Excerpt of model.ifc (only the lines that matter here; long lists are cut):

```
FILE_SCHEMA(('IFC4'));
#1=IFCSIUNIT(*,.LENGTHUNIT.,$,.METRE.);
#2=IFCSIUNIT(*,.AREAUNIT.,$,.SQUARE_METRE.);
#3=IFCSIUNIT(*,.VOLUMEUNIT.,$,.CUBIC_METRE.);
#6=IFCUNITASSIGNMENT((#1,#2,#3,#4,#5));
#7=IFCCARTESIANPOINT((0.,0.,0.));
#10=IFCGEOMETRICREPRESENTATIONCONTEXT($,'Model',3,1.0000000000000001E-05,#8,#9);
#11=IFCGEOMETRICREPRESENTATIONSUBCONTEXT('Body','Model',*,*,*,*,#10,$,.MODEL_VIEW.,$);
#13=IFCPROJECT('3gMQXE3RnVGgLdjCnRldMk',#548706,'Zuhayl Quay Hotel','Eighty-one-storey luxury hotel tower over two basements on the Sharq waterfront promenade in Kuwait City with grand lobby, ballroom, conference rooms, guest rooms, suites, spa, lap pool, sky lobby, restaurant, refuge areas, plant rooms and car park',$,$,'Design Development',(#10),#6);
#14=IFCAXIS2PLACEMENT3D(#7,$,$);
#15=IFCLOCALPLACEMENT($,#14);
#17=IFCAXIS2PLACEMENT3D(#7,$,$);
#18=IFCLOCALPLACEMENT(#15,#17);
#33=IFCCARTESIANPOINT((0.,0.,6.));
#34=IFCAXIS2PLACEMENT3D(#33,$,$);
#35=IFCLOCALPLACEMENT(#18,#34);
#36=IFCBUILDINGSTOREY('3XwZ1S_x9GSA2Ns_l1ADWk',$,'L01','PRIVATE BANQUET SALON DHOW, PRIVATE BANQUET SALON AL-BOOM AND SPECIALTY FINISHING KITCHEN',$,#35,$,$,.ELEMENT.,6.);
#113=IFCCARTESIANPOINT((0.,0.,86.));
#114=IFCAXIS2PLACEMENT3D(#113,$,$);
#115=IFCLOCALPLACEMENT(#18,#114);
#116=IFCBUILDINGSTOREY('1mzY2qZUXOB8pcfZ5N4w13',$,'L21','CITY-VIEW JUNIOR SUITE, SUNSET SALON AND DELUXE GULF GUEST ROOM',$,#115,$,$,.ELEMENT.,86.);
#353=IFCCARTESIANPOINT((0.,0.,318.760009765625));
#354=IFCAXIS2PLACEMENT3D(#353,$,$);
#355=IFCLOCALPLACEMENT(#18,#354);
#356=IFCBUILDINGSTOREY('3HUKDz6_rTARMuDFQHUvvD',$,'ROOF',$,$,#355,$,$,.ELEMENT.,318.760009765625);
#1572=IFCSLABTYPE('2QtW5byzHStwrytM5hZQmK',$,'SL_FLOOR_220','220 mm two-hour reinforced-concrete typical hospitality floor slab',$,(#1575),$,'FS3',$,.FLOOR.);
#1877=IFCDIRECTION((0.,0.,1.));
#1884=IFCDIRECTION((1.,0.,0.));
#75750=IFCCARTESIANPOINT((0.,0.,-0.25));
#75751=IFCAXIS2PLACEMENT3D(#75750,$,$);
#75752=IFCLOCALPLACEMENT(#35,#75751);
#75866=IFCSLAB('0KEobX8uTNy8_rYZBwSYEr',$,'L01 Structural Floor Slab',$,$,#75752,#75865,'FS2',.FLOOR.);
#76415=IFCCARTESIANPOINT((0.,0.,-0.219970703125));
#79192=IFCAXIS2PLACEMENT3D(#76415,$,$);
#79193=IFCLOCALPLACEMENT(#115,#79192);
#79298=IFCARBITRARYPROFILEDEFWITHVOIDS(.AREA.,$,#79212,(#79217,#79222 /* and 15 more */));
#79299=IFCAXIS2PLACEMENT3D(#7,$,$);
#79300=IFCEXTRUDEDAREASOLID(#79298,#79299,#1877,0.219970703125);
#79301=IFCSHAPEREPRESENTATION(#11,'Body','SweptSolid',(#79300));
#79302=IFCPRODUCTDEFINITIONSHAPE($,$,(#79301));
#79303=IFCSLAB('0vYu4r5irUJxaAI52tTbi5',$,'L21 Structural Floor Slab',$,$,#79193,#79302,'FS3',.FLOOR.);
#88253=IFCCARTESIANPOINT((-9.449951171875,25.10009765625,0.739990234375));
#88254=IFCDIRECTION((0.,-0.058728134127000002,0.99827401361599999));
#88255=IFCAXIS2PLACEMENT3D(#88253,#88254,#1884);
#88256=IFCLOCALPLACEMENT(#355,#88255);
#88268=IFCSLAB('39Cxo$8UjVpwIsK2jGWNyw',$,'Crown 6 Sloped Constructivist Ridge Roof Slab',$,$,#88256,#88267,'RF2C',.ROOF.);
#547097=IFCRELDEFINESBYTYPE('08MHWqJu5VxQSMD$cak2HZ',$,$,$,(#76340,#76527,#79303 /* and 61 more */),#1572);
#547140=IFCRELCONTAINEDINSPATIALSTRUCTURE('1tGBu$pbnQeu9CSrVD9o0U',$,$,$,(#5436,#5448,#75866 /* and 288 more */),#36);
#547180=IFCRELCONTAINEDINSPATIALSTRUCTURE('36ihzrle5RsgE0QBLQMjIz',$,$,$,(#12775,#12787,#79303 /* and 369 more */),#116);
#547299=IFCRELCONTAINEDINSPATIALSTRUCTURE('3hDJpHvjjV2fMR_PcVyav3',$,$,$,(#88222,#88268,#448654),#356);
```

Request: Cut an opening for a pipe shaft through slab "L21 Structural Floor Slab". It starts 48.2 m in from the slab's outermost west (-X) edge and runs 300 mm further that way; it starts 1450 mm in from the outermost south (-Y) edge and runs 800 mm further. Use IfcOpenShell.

```python
import numpy as np
import ifcopenshell
import ifcopenshell.api.feature
import ifcopenshell.api.geometry
import ifcopenshell.api.root
import ifcopenshell.geom
import ifcopenshell.util.placement
import ifcopenshell.util.representation
import ifcopenshell.util.shape
import ifcopenshell.util.unit

model = ifcopenshell.open("model.ifc")
unit_scale = ifcopenshell.util.unit.calculate_unit_scale(model)
settings = ifcopenshell.geom.settings()


def volume(element):
    """Net volume in cubic metres, openings subtracted."""
    shape = ifcopenshell.geom.create_shape(settings, element)
    return ifcopenshell.util.shape.get_volume(shape.geometry)


slab = model.by_guid("0vYu4r5irUJxaAI52tTbi5")
before = volume(slab)

# Extent in the slab's own axes, in metres. The edges named are its -X and -Y sides.
slab_shape = ifcopenshell.geom.create_shape(settings, slab)
vertices = ifcopenshell.util.shape.get_vertices(slab_shape.geometry)
x_min, y_min, bottom = vertices.min(axis=0)
top = vertices[:, 2].max()

opening = ifcopenshell.api.root.create_entity(model, ifc_class="IfcOpeningElement", name="Pipe shaft opening", predefined_type="OPENING")
context = ifcopenshell.util.representation.get_context(model, "Model", "Body", "MODEL_VIEW")
width, depth = 0.3, 0.8
outline = [(0.0, 0.0), (width, 0.0), (width, depth), (0.0, depth), (0.0, 0.0)]
# Overshoot both faces by 50 mm so the cut is clean.
shape = ifcopenshell.api.geometry.add_slab_representation(
    model, context=context, depth=top - bottom + 0.1, polyline=outline
)
ifcopenshell.api.geometry.assign_representation(model, product=opening, representation=shape)

matrix = ifcopenshell.util.placement.get_local_placement(slab.ObjectPlacement)
matrix[:, 3] = matrix @ np.append(np.array([x_min + 48.2, y_min + 1.45, bottom - 0.05]) / unit_scale, 1.0)
ifcopenshell.api.geometry.edit_object_placement(model, product=opening, matrix=matrix, is_si=False)
ifcopenshell.api.feature.add_feature(model, feature=opening, element=slab)

after = volume(slab)

print(f"slab volume {before:.3f} -> {after:.3f} m3")

model.write("model_rev.ifc")
```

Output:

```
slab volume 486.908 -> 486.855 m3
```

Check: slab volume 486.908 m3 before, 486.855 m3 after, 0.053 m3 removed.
